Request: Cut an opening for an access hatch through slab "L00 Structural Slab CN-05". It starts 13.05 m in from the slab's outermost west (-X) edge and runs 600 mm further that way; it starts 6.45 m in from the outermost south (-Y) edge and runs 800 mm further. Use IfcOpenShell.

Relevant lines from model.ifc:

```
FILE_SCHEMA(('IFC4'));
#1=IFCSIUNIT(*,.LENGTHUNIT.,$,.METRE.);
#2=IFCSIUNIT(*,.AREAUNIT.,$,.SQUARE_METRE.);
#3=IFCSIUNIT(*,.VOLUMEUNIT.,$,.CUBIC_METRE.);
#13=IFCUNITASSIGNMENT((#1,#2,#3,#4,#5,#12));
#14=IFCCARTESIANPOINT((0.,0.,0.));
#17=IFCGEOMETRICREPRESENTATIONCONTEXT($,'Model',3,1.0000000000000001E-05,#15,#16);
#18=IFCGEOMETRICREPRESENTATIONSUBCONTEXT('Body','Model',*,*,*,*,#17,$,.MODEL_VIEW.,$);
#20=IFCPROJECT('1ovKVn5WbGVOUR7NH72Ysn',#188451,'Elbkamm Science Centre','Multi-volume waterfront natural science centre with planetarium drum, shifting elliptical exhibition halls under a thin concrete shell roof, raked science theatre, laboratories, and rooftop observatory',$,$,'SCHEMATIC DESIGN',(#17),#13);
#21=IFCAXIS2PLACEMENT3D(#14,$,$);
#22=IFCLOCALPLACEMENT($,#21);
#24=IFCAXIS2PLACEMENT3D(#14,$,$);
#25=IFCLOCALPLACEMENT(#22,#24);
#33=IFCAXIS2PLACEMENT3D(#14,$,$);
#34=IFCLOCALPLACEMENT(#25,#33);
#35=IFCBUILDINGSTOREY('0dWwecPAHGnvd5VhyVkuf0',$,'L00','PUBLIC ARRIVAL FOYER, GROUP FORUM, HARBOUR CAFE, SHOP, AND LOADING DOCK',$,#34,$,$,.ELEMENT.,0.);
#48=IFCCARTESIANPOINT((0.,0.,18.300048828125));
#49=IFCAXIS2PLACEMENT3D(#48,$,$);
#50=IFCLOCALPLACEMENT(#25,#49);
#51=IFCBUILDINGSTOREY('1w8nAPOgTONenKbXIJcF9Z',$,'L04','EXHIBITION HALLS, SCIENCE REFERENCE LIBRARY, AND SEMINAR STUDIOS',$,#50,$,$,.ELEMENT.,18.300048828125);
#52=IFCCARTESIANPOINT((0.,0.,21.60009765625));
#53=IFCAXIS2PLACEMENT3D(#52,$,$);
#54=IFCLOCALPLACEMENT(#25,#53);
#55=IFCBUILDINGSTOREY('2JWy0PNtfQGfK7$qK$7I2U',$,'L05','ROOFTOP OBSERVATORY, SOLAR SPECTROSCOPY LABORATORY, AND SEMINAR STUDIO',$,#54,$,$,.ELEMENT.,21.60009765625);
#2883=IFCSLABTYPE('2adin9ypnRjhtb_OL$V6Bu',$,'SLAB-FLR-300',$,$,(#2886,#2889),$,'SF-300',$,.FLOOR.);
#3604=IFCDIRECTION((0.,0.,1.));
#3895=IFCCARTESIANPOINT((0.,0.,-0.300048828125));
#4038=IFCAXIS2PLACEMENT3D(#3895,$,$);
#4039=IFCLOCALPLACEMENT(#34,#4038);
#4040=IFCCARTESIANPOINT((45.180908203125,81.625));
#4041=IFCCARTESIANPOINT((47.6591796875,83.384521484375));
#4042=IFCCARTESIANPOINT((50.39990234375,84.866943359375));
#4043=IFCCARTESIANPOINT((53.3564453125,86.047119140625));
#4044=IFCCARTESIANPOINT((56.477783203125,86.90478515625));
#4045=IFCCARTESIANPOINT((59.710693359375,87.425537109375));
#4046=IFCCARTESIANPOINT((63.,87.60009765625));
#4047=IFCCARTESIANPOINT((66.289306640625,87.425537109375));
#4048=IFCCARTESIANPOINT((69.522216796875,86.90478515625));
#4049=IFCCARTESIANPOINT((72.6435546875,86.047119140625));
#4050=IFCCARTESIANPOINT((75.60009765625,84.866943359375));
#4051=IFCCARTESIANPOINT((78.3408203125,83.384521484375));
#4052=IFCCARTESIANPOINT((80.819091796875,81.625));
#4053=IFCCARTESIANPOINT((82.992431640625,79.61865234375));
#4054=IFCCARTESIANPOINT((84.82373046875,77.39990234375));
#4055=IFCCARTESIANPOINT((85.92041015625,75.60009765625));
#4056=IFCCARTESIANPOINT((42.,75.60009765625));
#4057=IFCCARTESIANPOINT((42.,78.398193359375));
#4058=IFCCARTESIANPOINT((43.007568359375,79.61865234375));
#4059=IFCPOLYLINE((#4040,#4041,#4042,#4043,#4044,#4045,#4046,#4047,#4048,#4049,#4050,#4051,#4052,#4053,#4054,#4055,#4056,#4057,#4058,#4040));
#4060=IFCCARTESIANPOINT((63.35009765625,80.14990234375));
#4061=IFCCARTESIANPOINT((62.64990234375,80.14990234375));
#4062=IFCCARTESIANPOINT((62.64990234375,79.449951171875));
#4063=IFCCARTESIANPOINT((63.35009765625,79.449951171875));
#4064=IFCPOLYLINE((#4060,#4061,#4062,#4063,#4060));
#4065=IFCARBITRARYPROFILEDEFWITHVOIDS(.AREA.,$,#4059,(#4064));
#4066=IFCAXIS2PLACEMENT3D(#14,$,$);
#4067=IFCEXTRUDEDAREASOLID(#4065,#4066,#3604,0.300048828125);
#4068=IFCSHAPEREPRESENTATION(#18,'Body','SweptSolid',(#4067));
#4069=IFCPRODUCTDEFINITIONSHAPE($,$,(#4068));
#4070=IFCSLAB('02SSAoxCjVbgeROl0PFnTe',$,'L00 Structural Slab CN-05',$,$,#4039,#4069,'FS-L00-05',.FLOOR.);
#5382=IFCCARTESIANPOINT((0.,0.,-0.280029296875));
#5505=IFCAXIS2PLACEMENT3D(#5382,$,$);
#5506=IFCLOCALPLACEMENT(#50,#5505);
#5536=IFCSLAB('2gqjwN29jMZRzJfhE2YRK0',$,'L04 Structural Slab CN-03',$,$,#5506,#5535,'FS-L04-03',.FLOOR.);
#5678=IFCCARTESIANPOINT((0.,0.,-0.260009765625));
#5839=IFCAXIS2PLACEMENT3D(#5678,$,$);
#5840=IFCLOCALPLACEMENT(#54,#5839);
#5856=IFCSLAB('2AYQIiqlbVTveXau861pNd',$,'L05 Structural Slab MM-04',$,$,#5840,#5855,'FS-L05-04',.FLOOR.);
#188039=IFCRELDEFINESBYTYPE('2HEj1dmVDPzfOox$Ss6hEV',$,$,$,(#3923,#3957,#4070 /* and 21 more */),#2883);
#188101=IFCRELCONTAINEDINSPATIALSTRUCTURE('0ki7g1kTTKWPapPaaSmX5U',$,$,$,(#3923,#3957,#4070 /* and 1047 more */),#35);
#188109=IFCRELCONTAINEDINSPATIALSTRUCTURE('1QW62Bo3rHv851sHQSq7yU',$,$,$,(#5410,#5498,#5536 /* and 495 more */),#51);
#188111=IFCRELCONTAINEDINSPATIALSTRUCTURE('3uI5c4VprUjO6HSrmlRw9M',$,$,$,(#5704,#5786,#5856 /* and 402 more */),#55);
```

```python
import numpy as np
import ifcopenshell
import ifcopenshell.api.feature
import ifcopenshell.api.geometry
import ifcopenshell.api.root
import ifcopenshell.geom
import ifcopenshell.util.placement
import ifcopenshell.util.representation
import ifcopenshell.util.shape
import ifcopenshell.util.unit

model = ifcopenshell.open("model.ifc")
unit_scale = ifcopenshell.util.unit.calculate_unit_scale(model)
settings = ifcopenshell.geom.settings()


def volume(element):
    """Net volume in cubic metres, openings subtracted."""
    shape = ifcopenshell.geom.create_shape(settings, element)
    return ifcopenshell.util.shape.get_volume(shape.geometry)


slab = model.by_id(4070)
before = volume(slab)

# Extent in the slab's own axes, in metres. The edges named are its -X and -Y sides.
slab_shape = ifcopenshell.geom.create_shape(settings, slab)
vertices = ifcopenshell.util.shape.get_vertices(slab_shape.geometry)
x_min, y_min, bottom = vertices.min(axis=0)
top = vertices[:, 2].max()

opening = ifcopenshell.api.root.create_entity(model, ifc_class="IfcOpeningElement", name="Access hatch opening", predefined_type="OPENING")
context = ifcopenshell.util.representation.get_context(model, "Model", "Body", "MODEL_VIEW")
width, depth = 0.6, 0.8
outline = [(0.0, 0.0), (width, 0.0), (width, depth), (0.0, depth), (0.0, 0.0)]
# Overshoot both faces by 50 mm so the cut is clean.
shape = ifcopenshell.api.geometry.add_slab_representation(
    model, context=context, depth=top - bottom + 0.1, polyline=outline
)
ifcopenshell.api.geometry.assign_representation(model, product=opening, representation=shape)

matrix = ifcopenshell.util.placement.get_local_placement(slab.ObjectPlacement)
matrix[:, 3] = matrix @ np.append(np.array([x_min + 13.05, y_min + 6.45, bottom - 0.05]) / unit_scale, 1.0)
ifcopenshell.api.geometry.edit_object_placement(model, product=opening, matrix=matrix, is_si=False)
ifcopenshell.api.feature.add_feature(model, feature=opening, element=slab)

after = volume(slab)

print(f"slab volume {before:.3f} -> {after:.3f} m3")

model.write("model-out.ifc")
```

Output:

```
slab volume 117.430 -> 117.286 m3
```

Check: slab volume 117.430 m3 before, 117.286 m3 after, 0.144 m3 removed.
